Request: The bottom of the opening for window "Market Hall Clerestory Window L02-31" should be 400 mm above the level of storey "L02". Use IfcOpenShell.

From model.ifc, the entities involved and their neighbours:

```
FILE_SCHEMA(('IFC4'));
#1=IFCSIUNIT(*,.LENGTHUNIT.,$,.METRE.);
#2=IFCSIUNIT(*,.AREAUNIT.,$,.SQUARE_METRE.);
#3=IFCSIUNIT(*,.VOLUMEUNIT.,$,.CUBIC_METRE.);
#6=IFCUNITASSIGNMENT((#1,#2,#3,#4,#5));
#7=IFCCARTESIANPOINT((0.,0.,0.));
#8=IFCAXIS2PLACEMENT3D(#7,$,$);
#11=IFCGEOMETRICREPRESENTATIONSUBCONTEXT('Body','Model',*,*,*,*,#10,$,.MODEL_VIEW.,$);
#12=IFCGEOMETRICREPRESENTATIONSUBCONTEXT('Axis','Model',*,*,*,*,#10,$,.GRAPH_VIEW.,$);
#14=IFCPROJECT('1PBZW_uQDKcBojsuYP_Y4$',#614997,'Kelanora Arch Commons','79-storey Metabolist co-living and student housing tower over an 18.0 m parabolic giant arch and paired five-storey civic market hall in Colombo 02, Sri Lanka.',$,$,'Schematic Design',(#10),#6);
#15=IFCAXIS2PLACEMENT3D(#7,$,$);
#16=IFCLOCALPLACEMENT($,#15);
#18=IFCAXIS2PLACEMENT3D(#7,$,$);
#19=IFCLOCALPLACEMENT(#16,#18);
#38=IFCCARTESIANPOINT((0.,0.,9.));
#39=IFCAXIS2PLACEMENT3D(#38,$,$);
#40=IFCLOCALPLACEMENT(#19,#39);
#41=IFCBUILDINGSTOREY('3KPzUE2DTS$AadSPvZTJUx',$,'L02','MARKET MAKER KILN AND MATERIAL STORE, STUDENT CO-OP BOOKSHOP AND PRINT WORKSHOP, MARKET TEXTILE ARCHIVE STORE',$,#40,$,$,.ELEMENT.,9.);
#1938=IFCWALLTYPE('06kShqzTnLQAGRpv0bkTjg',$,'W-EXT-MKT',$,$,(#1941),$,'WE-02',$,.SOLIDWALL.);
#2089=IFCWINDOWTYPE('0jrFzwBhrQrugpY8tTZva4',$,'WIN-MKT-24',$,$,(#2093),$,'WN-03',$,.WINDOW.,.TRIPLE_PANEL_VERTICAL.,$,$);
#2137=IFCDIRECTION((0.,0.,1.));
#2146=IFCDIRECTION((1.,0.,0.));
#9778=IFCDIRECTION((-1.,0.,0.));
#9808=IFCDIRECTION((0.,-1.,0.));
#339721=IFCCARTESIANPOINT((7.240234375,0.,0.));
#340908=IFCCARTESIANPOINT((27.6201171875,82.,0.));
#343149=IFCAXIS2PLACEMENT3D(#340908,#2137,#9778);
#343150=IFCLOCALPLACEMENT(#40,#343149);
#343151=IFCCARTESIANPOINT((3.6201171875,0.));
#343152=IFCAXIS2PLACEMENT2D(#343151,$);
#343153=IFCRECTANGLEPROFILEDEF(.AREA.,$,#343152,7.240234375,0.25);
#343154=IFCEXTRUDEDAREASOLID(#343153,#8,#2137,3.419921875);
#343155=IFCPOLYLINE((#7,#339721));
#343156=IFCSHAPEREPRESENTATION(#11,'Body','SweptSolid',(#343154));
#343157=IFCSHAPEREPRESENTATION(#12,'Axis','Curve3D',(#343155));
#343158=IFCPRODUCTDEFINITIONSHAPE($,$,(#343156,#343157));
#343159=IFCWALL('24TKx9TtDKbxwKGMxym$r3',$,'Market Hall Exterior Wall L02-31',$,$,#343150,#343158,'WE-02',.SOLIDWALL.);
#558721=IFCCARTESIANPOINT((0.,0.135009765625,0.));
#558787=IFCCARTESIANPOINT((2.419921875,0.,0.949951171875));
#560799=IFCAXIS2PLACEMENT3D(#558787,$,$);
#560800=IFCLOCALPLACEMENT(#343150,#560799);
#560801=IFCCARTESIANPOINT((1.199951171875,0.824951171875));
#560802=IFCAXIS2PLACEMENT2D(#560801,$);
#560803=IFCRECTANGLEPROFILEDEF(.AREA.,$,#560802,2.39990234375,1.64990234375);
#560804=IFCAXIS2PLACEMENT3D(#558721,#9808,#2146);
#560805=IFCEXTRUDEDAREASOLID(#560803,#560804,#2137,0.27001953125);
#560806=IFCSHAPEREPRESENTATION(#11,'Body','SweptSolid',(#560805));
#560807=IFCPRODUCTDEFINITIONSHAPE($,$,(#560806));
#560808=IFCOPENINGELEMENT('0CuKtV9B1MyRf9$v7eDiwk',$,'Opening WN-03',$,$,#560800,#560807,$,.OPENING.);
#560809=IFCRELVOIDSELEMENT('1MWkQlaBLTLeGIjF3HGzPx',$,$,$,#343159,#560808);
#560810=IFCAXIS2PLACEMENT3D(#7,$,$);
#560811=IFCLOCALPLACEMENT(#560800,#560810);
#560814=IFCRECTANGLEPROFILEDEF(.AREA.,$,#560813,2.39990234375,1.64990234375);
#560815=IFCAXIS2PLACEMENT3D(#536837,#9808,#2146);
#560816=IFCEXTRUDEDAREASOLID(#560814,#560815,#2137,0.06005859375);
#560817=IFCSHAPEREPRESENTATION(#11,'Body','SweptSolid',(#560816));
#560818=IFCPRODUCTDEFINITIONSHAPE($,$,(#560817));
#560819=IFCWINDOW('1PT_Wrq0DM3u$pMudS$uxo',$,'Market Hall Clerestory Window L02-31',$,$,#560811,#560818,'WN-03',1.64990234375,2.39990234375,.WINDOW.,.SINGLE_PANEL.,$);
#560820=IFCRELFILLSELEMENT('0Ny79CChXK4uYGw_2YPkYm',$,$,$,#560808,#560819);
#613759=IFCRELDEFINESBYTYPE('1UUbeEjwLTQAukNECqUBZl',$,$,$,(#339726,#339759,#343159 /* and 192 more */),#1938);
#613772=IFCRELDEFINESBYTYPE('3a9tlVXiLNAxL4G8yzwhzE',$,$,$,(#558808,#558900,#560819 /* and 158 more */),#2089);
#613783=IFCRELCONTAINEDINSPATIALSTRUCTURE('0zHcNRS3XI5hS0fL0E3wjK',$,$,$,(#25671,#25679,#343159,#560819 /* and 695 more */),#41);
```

```python
import numpy as np
import ifcopenshell
import ifcopenshell.api.geometry
import ifcopenshell.geom
import ifcopenshell.util.element
import ifcopenshell.util.placement
import ifcopenshell.util.shape
import ifcopenshell.util.unit

model = ifcopenshell.open("model.ifc")
unit_scale = ifcopenshell.util.unit.calculate_unit_scale(model)

window = model.by_id(560819)
opening = window.FillsVoids[0].RelatingOpeningElement
storey = ifcopenshell.util.element.get_container(window, ifc_class="IfcBuildingStorey")
level = ifcopenshell.util.placement.get_local_placement(storey.ObjectPlacement)[2, 3]

# The opening's origin need not be at the sill, so measure its lowest point.
shape = ifcopenshell.geom.create_shape(ifcopenshell.geom.settings(), opening)
bottom = ifcopenshell.util.shape.get_shape_bottom_elevation(shape, shape.geometry) / unit_scale
dz = level + 0.4 / unit_scale - bottom

shift = np.array([0.0, 0.0, dz])
# The window is placed relative to its opening, so it follows when the opening moves.
matrix = ifcopenshell.util.placement.get_local_placement(opening.ObjectPlacement)
matrix[:3, 3] += shift
ifcopenshell.api.geometry.edit_object_placement(
    model, product=opening, matrix=matrix, is_si=False, should_transform_children=True
)

print(f"moved by {dz * unit_scale:+.3f} m")

model.write("model_edited.ifc")
```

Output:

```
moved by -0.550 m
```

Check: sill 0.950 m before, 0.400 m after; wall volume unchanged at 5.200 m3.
